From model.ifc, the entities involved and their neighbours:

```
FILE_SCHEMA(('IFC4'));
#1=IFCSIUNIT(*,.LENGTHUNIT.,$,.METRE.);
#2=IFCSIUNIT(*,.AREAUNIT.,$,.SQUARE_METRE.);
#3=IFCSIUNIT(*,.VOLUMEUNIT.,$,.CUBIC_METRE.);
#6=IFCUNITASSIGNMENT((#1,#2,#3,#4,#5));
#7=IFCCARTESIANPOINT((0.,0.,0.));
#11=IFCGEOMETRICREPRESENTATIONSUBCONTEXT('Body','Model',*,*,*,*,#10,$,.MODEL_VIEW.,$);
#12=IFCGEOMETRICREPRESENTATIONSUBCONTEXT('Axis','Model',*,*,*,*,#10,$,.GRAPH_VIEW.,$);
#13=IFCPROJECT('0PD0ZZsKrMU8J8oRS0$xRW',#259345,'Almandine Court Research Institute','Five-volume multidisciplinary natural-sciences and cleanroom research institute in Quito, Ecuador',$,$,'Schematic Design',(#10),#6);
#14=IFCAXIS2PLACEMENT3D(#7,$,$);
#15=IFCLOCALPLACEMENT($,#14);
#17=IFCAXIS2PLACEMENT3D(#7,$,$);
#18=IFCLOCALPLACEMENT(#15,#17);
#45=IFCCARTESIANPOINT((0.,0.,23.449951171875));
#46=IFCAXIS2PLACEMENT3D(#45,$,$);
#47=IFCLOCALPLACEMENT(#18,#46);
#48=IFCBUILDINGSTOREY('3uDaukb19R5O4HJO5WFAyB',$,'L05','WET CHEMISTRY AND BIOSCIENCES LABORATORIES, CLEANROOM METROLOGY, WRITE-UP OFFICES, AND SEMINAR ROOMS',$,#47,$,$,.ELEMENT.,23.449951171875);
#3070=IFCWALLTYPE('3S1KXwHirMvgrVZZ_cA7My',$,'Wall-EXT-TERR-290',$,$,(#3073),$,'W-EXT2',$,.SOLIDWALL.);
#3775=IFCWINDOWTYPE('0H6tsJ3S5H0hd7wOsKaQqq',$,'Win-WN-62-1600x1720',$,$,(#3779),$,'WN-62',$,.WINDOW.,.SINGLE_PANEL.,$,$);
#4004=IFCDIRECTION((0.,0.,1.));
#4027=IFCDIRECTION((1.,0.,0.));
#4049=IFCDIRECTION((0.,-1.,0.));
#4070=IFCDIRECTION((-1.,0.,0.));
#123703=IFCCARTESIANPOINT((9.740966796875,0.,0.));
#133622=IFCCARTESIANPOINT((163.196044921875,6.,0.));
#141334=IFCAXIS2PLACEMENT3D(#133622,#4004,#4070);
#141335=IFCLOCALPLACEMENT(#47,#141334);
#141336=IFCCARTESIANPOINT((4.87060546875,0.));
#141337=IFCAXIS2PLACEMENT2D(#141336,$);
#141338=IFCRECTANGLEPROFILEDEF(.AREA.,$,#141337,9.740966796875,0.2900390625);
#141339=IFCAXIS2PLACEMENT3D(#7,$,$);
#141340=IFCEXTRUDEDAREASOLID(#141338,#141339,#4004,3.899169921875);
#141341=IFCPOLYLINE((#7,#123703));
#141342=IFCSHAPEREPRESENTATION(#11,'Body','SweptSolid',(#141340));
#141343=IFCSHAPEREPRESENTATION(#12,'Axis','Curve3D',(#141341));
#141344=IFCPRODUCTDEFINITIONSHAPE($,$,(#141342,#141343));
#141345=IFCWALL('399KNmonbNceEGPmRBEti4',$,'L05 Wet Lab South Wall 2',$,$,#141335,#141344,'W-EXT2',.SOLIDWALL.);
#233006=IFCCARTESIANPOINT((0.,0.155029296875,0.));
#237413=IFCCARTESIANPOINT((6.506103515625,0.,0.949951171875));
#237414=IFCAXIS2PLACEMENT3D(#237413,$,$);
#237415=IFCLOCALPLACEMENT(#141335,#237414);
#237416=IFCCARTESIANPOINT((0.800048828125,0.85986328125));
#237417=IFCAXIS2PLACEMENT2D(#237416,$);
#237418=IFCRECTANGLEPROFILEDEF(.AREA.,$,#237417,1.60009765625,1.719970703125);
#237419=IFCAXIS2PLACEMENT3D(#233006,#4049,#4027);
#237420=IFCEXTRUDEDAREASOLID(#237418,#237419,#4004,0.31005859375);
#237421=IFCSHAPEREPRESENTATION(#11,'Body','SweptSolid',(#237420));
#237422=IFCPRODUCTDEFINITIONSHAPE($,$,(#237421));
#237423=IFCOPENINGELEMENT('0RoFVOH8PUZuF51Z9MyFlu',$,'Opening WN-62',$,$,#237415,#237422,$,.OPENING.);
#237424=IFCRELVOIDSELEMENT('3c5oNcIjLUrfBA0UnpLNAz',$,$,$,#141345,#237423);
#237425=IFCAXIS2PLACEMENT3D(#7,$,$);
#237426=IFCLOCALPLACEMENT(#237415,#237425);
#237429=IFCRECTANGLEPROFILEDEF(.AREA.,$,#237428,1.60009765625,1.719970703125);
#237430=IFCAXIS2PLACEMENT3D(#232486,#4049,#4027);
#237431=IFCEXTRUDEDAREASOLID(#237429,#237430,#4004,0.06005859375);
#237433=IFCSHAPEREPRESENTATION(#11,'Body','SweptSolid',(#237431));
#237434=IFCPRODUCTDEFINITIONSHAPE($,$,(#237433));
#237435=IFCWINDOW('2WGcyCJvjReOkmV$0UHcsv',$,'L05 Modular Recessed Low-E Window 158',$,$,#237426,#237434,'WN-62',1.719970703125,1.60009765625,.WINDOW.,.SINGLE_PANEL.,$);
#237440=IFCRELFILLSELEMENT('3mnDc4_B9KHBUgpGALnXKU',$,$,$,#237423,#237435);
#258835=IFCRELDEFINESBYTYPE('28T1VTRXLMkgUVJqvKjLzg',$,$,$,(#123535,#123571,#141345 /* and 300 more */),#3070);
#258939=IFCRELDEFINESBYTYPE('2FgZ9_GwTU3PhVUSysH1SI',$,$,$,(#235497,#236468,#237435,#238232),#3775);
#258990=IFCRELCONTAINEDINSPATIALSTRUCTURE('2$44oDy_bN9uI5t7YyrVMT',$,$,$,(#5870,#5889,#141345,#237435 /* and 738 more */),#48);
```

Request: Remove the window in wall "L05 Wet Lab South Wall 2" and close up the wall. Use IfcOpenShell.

```python
import ifcopenshell
import ifcopenshell.api.feature
import ifcopenshell.api.root
import ifcopenshell.geom
import ifcopenshell.util.shape

model = ifcopenshell.open("model.ifc")
settings = ifcopenshell.geom.settings()


def volume(element):
    """Net volume in cubic metres, openings subtracted."""
    shape = ifcopenshell.geom.create_shape(settings, element)
    return ifcopenshell.util.shape.get_volume(shape.geometry)


window = model.by_guid("2WGcyCJvjReOkmV$0UHcsv")
opening = window.FillsVoids[0].RelatingOpeningElement
wall = opening.VoidsElements[0].RelatingBuildingElement
before = volume(wall)

ifcopenshell.api.root.remove_product(model, product=window)
ifcopenshell.api.feature.remove_feature(model, feature=opening)

after = volume(wall)

print(f"wall volume {before:.3f} -> {after:.3f} m3")

model.write("model-out.ifc")
```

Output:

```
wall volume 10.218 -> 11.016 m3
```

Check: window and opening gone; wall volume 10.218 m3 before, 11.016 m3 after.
